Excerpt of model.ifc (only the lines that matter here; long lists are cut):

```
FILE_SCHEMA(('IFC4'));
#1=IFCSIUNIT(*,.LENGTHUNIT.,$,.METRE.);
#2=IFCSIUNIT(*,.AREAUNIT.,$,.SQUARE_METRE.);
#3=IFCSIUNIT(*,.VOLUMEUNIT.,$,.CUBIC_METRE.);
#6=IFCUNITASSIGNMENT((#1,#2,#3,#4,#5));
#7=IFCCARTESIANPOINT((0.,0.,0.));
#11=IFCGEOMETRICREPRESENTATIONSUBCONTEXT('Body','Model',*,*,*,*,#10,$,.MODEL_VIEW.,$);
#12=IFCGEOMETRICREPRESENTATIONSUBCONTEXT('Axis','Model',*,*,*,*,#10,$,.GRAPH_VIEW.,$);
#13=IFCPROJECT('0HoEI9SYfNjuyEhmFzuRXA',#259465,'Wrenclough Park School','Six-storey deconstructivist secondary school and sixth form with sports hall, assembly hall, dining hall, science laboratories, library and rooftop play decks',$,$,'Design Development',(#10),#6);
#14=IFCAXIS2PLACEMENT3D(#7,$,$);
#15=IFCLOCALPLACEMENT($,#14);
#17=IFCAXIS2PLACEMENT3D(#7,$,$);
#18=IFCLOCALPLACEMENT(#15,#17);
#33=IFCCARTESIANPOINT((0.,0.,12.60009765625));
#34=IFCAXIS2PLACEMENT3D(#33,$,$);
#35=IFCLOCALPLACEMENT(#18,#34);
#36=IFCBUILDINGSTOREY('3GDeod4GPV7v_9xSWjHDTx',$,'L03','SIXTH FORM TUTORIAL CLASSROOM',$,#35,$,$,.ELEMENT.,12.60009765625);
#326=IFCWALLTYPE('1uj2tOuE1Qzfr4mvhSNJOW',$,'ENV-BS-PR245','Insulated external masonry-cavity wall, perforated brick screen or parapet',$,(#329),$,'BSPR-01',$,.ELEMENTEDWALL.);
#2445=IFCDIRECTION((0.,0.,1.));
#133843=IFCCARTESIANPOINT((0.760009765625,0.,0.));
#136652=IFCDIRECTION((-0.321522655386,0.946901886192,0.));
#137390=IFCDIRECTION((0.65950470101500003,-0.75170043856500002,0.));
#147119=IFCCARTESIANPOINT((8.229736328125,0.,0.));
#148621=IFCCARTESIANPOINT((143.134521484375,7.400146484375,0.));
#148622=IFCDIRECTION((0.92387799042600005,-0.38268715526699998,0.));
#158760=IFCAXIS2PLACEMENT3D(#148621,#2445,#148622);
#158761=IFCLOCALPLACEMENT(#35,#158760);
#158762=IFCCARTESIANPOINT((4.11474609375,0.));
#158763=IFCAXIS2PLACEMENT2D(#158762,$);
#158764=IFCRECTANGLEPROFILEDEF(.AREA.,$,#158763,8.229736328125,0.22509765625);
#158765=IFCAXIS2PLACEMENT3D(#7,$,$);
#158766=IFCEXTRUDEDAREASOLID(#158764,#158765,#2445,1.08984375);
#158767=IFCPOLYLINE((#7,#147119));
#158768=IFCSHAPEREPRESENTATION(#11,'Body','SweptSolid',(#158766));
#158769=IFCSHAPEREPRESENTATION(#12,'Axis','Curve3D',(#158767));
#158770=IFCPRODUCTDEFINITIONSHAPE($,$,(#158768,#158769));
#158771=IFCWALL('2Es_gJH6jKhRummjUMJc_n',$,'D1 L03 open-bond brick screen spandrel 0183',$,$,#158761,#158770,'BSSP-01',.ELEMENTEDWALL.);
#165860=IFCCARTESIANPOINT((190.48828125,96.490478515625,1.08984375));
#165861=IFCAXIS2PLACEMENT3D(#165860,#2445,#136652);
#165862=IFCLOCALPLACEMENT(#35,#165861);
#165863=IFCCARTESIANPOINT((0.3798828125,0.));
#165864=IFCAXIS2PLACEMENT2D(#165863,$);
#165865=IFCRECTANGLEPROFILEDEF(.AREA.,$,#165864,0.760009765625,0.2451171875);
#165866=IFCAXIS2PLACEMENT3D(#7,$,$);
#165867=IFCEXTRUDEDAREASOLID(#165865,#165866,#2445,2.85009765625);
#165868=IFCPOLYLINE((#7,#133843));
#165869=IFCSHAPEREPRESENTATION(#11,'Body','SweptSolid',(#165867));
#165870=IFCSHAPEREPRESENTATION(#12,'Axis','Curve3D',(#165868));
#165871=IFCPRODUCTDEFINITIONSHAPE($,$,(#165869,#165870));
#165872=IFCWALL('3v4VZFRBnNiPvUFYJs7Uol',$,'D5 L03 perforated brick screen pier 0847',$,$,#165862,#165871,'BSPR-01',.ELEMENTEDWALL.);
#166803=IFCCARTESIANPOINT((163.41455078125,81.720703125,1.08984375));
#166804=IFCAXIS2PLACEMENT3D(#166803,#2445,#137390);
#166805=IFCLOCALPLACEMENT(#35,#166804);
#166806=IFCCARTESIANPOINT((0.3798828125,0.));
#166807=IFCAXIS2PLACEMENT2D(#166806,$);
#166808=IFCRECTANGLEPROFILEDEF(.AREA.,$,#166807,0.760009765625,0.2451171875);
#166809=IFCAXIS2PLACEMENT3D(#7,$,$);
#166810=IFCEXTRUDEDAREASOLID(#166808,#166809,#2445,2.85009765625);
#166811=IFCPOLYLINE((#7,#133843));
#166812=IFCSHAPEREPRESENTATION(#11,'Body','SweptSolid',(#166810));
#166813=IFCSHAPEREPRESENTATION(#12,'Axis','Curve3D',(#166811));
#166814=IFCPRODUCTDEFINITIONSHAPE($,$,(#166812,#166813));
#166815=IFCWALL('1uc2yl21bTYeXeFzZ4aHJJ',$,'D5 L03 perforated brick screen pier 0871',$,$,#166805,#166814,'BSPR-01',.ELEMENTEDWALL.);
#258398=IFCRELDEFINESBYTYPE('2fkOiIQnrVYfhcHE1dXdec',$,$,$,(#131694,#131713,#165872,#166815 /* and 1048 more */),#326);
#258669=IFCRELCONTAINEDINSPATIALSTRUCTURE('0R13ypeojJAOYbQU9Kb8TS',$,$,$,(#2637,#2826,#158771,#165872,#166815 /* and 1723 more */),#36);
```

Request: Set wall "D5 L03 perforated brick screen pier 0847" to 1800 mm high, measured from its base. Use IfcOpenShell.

```python
import ifcopenshell
import ifcopenshell.geom
import ifcopenshell.util.representation
import ifcopenshell.util.shape
import ifcopenshell.util.unit

model = ifcopenshell.open("model.ifc")
unit_scale = ifcopenshell.util.unit.calculate_unit_scale(model)
settings = ifcopenshell.geom.settings()


def volume(element):
    """Net volume in cubic metres, openings subtracted."""
    shape = ifcopenshell.geom.create_shape(settings, element)
    return ifcopenshell.util.shape.get_volume(shape.geometry)


wall = model.by_guid("3v4VZFRBnNiPvUFYJs7Uol")
before = volume(wall)

body = ifcopenshell.util.representation.get_representation(wall, "Model", "Body")
solid = body.Items[0]
old_height = solid.Depth
solid.Depth = 1.8 / unit_scale
after = volume(wall)

print(f"height {old_height:g} -> {solid.Depth:g}, volume {before:.3f} -> {after:.3f} m3")

model.write("model-out.ifc")
```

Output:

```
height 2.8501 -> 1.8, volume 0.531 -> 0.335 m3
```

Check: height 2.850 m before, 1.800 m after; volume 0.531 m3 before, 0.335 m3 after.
